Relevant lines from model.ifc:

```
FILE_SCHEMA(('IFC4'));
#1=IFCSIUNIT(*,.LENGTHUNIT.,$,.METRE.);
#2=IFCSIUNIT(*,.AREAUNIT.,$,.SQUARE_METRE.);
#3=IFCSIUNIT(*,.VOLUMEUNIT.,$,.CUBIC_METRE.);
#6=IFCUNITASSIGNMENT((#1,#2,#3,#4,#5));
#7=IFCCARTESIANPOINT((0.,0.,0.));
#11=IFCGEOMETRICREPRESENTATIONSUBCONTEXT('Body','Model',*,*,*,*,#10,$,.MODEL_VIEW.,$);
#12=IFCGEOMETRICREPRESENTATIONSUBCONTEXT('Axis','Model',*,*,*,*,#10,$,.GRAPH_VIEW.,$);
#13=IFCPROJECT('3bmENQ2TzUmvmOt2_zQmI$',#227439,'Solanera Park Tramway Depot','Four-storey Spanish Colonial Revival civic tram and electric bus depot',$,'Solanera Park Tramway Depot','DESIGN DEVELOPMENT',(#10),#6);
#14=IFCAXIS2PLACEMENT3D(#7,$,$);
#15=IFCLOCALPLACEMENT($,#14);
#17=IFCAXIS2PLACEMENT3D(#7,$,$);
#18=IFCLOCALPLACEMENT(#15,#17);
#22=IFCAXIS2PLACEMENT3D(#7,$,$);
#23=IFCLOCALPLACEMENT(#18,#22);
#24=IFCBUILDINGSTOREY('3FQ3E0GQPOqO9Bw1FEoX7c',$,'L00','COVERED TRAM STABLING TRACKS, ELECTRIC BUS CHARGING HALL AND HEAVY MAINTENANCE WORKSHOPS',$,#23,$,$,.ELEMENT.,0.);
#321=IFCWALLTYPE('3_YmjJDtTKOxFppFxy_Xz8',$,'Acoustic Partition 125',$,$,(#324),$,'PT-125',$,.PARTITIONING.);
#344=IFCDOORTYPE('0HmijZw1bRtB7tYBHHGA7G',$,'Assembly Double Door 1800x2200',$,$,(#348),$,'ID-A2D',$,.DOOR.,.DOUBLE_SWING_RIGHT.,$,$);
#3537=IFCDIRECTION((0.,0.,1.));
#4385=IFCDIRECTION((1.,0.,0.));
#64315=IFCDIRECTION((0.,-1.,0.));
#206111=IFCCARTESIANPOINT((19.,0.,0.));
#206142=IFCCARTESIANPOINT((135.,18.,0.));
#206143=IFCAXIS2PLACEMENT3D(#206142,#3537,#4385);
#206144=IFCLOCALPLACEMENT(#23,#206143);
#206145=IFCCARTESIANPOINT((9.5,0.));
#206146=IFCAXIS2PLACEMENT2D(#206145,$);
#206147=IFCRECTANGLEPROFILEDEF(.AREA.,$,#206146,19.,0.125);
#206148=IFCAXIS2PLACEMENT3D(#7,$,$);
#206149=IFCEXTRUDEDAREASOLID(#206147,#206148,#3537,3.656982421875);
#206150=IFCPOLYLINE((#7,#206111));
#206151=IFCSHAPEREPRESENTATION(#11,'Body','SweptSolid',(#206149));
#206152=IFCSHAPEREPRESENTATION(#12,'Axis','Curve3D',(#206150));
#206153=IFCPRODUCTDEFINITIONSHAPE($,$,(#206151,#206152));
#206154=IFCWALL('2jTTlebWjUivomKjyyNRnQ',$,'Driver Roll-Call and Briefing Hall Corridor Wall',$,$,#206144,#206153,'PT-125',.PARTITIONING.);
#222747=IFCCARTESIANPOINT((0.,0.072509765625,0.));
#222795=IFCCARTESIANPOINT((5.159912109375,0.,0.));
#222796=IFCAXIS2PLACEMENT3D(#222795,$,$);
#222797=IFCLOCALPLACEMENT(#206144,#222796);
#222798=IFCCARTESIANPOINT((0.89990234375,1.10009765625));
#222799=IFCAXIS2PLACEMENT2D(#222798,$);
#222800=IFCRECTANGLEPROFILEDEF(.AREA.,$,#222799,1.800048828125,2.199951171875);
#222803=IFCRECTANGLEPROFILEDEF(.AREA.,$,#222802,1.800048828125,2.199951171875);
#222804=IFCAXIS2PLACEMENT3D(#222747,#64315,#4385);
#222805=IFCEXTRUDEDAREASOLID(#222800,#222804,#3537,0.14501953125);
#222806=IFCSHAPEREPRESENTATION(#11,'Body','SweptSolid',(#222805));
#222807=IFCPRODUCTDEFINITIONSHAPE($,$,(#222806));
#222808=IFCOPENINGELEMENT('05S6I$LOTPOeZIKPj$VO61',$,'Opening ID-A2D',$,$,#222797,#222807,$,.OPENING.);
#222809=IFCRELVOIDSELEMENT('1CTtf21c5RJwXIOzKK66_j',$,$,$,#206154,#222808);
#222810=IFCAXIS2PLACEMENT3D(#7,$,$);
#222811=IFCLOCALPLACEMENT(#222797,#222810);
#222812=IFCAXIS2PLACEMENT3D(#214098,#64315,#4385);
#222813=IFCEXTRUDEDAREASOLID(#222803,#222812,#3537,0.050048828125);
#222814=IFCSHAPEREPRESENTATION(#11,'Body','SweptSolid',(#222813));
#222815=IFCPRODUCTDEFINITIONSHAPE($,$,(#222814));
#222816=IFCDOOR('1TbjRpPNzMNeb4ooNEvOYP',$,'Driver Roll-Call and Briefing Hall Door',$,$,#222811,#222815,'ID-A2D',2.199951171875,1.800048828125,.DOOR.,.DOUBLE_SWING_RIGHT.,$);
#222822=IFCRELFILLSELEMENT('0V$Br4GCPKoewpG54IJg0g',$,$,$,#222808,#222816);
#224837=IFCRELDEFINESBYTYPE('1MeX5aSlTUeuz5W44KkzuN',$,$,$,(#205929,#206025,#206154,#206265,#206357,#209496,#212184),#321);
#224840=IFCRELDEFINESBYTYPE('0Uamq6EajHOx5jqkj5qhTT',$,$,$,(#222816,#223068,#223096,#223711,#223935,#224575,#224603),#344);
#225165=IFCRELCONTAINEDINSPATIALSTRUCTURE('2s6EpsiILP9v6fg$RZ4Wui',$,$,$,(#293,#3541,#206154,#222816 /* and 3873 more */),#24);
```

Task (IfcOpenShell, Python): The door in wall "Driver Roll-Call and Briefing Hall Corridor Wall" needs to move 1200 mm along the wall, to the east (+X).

```python
import ifcopenshell
import ifcopenshell.api.geometry
import ifcopenshell.util.placement

model = ifcopenshell.open("model.ifc")

door = model.by_guid("1TbjRpPNzMNeb4ooNEvOYP")
opening = door.FillsVoids[0].RelatingOpeningElement
wall = opening.VoidsElements[0].RelatingBuildingElement

wall_matrix = ifcopenshell.util.placement.get_local_placement(wall.ObjectPlacement)
shift = wall_matrix[:3, 0] * 1.2
before = ifcopenshell.util.placement.get_local_placement(door.ObjectPlacement)[:3, 3].copy()

# The door is placed relative to its opening, so it follows when the opening moves.
matrix = ifcopenshell.util.placement.get_local_placement(opening.ObjectPlacement)
matrix[:3, 3] += shift
ifcopenshell.api.geometry.edit_object_placement(
    model, product=opening, matrix=matrix, is_si=False, should_transform_children=True
)

after = ifcopenshell.util.placement.get_local_placement(door.ObjectPlacement)[:3, 3]
print("door moved by", (after - before).round(3) + 0.0)

model.write("model_v2.ifc")
```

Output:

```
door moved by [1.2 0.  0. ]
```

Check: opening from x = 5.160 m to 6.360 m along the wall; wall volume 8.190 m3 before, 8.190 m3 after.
